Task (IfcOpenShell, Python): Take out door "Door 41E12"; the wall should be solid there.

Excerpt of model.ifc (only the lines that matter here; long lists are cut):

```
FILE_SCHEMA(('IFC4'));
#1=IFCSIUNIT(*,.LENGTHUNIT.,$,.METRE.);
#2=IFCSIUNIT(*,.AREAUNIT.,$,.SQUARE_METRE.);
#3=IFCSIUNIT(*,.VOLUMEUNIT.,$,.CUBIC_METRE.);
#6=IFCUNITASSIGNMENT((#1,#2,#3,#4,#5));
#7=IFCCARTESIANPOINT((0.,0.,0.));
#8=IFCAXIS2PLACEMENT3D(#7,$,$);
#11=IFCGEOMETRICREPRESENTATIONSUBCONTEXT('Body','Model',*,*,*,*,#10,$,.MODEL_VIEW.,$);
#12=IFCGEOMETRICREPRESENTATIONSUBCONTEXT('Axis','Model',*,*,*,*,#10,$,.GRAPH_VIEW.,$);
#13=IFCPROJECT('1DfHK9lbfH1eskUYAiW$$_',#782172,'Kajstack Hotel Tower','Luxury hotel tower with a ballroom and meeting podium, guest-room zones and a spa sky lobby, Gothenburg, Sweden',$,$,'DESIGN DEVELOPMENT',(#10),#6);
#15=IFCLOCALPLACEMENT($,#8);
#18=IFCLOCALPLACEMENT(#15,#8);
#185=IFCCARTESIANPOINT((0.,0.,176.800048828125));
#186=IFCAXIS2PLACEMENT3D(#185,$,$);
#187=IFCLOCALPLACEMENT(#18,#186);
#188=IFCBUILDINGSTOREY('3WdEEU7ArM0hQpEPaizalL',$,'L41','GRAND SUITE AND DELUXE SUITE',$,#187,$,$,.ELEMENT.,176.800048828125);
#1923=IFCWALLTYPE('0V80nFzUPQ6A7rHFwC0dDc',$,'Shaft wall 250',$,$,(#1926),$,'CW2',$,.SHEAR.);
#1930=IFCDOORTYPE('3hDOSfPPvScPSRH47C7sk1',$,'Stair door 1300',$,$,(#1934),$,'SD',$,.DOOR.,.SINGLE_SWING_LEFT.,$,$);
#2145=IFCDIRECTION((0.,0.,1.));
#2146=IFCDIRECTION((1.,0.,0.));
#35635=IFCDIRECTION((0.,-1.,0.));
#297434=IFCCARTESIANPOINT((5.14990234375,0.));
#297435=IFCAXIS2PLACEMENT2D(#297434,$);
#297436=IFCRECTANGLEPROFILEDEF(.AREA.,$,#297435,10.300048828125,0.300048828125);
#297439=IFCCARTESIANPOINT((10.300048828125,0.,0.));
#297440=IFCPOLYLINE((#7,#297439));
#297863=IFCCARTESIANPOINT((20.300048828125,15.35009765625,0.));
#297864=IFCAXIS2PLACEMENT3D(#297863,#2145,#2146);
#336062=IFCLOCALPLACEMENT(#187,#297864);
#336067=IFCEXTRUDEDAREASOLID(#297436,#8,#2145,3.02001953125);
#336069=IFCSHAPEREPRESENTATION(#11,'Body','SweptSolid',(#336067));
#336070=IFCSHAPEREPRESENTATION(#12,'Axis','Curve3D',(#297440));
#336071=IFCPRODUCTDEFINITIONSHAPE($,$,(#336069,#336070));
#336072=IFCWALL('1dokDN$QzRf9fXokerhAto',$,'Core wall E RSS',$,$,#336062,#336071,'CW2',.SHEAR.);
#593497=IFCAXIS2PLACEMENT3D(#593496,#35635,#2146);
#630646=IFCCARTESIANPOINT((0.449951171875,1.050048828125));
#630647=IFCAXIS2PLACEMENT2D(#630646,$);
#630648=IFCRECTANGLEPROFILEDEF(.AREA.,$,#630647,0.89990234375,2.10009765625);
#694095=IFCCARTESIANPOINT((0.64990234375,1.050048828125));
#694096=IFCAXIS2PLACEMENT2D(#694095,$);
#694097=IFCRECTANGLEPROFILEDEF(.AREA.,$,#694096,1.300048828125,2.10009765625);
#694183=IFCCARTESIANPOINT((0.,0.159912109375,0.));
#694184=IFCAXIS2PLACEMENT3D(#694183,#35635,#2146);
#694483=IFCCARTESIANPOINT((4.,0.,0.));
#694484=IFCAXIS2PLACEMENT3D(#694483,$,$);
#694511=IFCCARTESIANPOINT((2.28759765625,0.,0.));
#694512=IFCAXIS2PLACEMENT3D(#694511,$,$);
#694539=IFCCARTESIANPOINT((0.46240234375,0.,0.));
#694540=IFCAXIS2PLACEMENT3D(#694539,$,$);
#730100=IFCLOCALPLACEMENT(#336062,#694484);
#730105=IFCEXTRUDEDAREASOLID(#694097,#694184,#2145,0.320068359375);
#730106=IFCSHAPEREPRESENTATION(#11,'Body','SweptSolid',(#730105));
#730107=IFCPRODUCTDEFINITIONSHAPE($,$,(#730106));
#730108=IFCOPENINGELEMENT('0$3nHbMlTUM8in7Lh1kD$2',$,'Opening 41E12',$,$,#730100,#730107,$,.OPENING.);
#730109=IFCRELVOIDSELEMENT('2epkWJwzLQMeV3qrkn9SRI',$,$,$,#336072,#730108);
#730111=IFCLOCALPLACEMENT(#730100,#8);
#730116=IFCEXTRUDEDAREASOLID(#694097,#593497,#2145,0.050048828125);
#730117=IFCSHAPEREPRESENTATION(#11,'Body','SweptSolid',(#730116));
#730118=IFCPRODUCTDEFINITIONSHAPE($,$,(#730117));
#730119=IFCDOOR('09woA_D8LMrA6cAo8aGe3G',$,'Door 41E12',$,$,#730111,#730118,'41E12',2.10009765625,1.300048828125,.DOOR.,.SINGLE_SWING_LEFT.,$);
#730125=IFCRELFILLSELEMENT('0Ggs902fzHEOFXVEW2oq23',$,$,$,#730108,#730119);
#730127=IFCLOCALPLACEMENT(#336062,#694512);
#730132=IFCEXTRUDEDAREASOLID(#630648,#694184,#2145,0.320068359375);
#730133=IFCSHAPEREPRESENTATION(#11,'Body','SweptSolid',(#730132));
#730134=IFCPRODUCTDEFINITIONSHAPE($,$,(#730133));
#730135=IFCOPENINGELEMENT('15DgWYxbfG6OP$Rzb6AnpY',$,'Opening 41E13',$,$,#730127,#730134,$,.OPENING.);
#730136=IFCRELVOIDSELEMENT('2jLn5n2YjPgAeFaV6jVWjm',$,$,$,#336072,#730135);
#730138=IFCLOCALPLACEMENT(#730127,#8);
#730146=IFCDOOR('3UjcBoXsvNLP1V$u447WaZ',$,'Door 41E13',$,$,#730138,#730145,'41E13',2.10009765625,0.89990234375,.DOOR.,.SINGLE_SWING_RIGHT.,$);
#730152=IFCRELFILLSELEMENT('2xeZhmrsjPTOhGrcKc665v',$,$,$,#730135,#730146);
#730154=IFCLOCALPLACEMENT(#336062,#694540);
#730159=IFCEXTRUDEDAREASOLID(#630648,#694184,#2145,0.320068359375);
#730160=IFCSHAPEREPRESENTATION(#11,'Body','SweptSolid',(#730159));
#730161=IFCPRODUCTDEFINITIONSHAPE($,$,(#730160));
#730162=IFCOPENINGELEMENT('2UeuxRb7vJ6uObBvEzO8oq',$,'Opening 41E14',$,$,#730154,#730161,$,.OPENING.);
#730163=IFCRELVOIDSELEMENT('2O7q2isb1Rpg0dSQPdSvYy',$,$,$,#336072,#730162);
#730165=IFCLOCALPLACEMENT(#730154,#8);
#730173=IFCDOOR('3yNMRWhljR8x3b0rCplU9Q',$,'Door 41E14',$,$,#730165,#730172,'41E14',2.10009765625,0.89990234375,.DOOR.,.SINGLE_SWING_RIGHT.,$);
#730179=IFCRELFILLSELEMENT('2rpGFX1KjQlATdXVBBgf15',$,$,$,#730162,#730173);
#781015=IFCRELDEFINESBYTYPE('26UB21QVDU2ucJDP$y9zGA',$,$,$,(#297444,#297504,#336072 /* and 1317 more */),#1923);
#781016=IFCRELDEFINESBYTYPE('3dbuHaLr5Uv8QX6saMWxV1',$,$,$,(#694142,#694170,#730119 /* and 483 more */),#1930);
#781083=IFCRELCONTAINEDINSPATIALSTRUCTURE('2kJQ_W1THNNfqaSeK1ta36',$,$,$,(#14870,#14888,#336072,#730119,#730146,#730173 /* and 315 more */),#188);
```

```python
import ifcopenshell
import ifcopenshell.api.feature
import ifcopenshell.api.root
import ifcopenshell.geom
import ifcopenshell.util.shape

model = ifcopenshell.open("model.ifc")
settings = ifcopenshell.geom.settings()


def volume(element):
    """Net volume in cubic metres, openings subtracted."""
    shape = ifcopenshell.geom.create_shape(settings, element)
    return ifcopenshell.util.shape.get_volume(shape.geometry)


door = model.by_guid("09woA_D8LMrA6cAo8aGe3G")
opening = door.FillsVoids[0].RelatingOpeningElement
wall = opening.VoidsElements[0].RelatingBuildingElement
before = volume(wall)

ifcopenshell.api.root.remove_product(model, product=door)
ifcopenshell.api.feature.remove_feature(model, feature=opening)

after = volume(wall)

print(f"wall volume {before:.3f} -> {after:.3f} m3")

model.write("model-out.ifc")
```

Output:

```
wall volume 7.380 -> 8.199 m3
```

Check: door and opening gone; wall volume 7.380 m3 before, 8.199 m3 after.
